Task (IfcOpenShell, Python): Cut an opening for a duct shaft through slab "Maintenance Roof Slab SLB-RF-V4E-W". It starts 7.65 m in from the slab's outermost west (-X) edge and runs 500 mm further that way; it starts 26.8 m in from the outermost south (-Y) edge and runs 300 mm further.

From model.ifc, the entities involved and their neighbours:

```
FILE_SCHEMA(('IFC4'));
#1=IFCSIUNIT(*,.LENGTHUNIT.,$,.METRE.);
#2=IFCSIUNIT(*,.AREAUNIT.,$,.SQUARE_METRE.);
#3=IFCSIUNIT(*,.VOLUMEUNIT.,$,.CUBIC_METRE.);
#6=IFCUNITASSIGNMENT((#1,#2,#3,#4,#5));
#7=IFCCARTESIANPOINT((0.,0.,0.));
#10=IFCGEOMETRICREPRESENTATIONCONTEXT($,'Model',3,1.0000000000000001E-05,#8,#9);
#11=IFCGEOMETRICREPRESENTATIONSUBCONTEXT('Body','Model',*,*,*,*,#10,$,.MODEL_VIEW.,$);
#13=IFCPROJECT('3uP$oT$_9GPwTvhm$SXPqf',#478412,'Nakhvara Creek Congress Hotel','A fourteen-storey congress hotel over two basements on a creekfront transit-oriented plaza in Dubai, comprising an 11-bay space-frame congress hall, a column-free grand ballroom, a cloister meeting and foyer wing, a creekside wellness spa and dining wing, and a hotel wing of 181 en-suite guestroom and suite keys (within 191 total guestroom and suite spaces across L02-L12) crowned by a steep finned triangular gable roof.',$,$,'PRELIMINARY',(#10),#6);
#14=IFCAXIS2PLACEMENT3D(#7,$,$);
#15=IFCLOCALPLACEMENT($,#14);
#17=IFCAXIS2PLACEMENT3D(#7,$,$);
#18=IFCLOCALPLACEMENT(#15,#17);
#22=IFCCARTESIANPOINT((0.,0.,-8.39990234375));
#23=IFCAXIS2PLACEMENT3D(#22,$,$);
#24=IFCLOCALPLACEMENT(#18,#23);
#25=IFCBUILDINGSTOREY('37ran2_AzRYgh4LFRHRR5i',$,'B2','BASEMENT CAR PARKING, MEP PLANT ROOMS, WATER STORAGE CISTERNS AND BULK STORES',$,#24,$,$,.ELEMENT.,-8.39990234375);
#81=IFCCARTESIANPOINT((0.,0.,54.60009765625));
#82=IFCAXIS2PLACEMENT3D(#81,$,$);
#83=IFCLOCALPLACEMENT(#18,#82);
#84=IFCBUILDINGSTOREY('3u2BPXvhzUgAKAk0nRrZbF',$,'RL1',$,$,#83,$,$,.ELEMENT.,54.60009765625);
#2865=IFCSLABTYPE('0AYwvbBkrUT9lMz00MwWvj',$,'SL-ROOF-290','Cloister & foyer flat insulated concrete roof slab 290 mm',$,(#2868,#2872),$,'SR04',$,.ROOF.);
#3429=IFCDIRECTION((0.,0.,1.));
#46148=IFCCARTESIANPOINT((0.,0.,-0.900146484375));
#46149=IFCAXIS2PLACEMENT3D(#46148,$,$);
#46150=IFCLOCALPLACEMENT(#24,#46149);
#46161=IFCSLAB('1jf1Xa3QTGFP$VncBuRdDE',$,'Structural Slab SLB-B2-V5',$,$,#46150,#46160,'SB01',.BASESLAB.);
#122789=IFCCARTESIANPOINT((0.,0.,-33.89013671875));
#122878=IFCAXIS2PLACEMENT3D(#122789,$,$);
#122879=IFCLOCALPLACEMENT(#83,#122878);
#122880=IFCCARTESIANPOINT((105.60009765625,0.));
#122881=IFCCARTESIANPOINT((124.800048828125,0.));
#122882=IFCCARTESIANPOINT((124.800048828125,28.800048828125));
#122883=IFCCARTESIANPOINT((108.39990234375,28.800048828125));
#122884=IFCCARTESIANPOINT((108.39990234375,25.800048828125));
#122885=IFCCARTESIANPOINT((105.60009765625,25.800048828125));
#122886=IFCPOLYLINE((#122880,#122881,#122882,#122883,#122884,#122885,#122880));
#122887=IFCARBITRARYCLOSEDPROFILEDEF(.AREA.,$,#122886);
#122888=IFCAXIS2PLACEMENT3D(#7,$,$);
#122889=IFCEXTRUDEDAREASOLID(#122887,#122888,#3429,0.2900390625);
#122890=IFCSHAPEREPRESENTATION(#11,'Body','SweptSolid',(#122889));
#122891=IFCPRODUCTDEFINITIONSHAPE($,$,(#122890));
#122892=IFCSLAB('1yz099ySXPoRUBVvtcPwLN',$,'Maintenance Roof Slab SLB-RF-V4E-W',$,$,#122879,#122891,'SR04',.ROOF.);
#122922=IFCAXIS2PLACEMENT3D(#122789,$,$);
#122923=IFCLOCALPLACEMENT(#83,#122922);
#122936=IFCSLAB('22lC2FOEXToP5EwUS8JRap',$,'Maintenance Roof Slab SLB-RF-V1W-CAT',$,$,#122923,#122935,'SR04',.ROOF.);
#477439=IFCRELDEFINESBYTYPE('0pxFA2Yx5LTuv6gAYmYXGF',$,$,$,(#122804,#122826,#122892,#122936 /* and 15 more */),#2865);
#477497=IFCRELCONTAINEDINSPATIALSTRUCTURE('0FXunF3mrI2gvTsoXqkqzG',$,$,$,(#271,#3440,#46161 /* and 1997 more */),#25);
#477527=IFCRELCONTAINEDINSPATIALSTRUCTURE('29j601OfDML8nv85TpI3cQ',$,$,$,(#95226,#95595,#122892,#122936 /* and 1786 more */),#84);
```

```python
import numpy as np
import ifcopenshell
import ifcopenshell.api.feature
import ifcopenshell.api.geometry
import ifcopenshell.api.root
import ifcopenshell.geom
import ifcopenshell.util.placement
import ifcopenshell.util.representation
import ifcopenshell.util.shape
import ifcopenshell.util.unit

model = ifcopenshell.open("model.ifc")
unit_scale = ifcopenshell.util.unit.calculate_unit_scale(model)
settings = ifcopenshell.geom.settings()


def volume(element):
    """Net volume in cubic metres, openings subtracted."""
    shape = ifcopenshell.geom.create_shape(settings, element)
    return ifcopenshell.util.shape.get_volume(shape.geometry)


slab = model.by_id(122892)
before = volume(slab)

# Extent in the slab's own axes, in metres. The edges named are its -X and -Y sides.
slab_shape = ifcopenshell.geom.create_shape(settings, slab)
vertices = ifcopenshell.util.shape.get_vertices(slab_shape.geometry)
x_min, y_min, bottom = vertices.min(axis=0)
top = vertices[:, 2].max()

opening = ifcopenshell.api.root.create_entity(model, ifc_class="IfcOpeningElement", name="Duct shaft opening", predefined_type="OPENING")
context = ifcopenshell.util.representation.get_context(model, "Model", "Body", "MODEL_VIEW")
width, depth = 0.5, 0.3
outline = [(0.0, 0.0), (width, 0.0), (width, depth), (0.0, depth), (0.0, 0.0)]
# Overshoot both faces by 50 mm so the cut is clean.
shape = ifcopenshell.api.geometry.add_slab_representation(
    model, context=context, depth=top - bottom + 0.1, polyline=outline
)
ifcopenshell.api.geometry.assign_representation(model, product=opening, representation=shape)

matrix = ifcopenshell.util.placement.get_local_placement(slab.ObjectPlacement)
matrix[:, 3] = matrix @ np.append(np.array([x_min + 7.65, y_min + 26.8, bottom - 0.05]) / unit_scale, 1.0)
ifcopenshell.api.geometry.edit_object_placement(model, product=opening, matrix=matrix, is_si=False)
ifcopenshell.api.feature.add_feature(model, feature=opening, element=slab)

after = volume(slab)

print(f"slab volume {before:.3f} -> {after:.3f} m3")

model.write("model_edited.ifc")
```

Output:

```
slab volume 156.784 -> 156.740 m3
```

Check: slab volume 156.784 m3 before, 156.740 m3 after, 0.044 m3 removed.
